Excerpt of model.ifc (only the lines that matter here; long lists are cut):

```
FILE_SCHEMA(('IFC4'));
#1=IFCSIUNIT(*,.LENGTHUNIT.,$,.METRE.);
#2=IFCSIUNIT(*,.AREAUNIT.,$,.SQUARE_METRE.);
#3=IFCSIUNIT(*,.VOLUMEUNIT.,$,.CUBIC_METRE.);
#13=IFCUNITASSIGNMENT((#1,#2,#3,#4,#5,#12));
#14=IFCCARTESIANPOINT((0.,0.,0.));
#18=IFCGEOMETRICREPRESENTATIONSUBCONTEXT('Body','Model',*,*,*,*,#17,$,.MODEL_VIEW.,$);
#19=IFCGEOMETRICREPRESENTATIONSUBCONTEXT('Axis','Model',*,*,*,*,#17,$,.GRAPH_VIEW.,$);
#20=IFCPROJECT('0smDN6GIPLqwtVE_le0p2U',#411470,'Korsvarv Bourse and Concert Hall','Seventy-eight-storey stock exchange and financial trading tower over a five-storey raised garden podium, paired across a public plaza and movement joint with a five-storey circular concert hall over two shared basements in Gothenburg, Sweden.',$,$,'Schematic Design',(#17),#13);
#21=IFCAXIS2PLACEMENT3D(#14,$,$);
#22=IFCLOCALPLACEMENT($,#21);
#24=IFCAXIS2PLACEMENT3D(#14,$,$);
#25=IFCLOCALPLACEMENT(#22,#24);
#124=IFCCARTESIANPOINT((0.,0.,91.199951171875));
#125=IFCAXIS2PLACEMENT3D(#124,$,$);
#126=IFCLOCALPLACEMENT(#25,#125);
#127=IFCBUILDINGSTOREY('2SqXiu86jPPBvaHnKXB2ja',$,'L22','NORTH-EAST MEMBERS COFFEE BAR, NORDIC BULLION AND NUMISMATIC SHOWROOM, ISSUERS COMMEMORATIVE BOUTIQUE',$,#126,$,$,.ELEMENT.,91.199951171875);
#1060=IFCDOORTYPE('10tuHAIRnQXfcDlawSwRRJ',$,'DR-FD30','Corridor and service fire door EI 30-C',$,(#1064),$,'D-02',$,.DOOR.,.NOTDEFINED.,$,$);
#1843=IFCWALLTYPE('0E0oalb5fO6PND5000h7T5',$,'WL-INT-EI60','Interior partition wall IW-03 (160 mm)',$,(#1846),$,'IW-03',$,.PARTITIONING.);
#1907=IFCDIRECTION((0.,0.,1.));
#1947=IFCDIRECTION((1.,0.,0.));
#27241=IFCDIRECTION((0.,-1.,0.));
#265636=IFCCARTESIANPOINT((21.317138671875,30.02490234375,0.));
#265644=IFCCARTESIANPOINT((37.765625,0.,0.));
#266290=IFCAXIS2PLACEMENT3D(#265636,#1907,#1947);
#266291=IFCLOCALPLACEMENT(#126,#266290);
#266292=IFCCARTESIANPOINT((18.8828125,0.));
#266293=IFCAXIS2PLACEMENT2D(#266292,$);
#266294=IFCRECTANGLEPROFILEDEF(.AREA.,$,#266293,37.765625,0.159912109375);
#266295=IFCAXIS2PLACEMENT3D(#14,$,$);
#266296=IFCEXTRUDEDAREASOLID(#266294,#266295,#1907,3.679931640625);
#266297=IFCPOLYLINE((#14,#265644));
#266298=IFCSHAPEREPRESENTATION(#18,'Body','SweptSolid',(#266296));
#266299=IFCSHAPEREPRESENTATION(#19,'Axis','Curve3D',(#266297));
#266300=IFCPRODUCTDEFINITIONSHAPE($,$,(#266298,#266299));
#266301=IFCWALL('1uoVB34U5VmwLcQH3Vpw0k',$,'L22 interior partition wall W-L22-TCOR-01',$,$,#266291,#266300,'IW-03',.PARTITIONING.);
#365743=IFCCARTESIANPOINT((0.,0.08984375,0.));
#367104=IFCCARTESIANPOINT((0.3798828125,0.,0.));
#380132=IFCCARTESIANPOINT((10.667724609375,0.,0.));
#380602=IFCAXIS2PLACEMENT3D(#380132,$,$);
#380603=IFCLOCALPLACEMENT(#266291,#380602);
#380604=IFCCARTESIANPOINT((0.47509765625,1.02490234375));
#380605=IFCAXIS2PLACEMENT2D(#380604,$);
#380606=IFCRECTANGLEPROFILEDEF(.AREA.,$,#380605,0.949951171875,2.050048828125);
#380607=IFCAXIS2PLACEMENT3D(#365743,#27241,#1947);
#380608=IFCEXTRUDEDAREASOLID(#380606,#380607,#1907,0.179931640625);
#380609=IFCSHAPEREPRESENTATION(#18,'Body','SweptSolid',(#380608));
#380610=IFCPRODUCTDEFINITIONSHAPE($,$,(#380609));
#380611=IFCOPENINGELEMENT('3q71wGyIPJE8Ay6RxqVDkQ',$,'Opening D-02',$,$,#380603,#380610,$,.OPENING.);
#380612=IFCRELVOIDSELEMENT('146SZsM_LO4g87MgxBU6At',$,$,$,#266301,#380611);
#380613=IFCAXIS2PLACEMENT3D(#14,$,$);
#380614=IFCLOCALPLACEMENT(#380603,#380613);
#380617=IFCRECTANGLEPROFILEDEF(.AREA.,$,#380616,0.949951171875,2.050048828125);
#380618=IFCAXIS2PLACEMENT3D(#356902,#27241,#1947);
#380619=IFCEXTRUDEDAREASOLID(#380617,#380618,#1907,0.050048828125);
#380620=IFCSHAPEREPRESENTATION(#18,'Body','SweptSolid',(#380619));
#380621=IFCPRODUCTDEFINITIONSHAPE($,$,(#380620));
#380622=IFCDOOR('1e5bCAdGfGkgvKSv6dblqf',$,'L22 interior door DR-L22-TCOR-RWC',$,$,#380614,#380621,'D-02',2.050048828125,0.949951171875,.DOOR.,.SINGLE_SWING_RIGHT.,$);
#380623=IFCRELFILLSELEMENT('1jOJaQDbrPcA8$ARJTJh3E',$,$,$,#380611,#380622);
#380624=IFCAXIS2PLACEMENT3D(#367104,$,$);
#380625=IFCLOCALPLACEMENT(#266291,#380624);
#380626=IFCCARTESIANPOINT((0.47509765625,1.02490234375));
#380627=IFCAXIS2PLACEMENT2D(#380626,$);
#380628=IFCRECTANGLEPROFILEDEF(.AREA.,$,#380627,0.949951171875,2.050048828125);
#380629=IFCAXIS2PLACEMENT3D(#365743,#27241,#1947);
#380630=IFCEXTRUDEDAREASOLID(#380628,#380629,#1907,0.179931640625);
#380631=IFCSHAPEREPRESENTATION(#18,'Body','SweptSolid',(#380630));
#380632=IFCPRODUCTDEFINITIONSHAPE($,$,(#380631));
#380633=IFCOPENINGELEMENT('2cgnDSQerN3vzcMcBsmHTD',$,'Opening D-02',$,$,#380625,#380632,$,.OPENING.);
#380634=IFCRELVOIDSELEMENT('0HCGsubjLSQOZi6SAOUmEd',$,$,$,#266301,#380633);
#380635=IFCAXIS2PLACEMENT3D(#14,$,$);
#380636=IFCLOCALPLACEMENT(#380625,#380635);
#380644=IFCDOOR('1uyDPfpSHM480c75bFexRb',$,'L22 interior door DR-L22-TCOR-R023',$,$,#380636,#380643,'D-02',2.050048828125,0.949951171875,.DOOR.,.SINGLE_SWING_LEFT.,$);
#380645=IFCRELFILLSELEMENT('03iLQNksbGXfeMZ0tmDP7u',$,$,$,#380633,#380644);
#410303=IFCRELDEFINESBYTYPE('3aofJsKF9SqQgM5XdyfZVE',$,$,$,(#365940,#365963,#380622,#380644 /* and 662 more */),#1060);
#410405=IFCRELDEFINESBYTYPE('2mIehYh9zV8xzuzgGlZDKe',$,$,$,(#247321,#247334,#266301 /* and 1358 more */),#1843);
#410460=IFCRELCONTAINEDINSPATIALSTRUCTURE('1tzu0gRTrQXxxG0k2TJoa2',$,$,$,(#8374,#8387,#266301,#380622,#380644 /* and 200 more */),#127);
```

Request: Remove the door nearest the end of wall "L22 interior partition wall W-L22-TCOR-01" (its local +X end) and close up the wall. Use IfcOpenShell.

```python
import ifcopenshell
import ifcopenshell.api.feature
import ifcopenshell.api.root
import ifcopenshell.geom
import ifcopenshell.util.shape

model = ifcopenshell.open("model.ifc")
settings = ifcopenshell.geom.settings()


def volume(element):
    """Net volume in cubic metres, openings subtracted."""
    shape = ifcopenshell.geom.create_shape(settings, element)
    return ifcopenshell.util.shape.get_volume(shape.geometry)


door = model.by_guid("1e5bCAdGfGkgvKSv6dblqf")
opening = door.FillsVoids[0].RelatingOpeningElement
wall = opening.VoidsElements[0].RelatingBuildingElement
before = volume(wall)

ifcopenshell.api.root.remove_product(model, product=door)
ifcopenshell.api.feature.remove_feature(model, feature=opening)

after = volume(wall)

print(f"wall volume {before:.3f} -> {after:.3f} m3")

model.write("model-out.ifc")
```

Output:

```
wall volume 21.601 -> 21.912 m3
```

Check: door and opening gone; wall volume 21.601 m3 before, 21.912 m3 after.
